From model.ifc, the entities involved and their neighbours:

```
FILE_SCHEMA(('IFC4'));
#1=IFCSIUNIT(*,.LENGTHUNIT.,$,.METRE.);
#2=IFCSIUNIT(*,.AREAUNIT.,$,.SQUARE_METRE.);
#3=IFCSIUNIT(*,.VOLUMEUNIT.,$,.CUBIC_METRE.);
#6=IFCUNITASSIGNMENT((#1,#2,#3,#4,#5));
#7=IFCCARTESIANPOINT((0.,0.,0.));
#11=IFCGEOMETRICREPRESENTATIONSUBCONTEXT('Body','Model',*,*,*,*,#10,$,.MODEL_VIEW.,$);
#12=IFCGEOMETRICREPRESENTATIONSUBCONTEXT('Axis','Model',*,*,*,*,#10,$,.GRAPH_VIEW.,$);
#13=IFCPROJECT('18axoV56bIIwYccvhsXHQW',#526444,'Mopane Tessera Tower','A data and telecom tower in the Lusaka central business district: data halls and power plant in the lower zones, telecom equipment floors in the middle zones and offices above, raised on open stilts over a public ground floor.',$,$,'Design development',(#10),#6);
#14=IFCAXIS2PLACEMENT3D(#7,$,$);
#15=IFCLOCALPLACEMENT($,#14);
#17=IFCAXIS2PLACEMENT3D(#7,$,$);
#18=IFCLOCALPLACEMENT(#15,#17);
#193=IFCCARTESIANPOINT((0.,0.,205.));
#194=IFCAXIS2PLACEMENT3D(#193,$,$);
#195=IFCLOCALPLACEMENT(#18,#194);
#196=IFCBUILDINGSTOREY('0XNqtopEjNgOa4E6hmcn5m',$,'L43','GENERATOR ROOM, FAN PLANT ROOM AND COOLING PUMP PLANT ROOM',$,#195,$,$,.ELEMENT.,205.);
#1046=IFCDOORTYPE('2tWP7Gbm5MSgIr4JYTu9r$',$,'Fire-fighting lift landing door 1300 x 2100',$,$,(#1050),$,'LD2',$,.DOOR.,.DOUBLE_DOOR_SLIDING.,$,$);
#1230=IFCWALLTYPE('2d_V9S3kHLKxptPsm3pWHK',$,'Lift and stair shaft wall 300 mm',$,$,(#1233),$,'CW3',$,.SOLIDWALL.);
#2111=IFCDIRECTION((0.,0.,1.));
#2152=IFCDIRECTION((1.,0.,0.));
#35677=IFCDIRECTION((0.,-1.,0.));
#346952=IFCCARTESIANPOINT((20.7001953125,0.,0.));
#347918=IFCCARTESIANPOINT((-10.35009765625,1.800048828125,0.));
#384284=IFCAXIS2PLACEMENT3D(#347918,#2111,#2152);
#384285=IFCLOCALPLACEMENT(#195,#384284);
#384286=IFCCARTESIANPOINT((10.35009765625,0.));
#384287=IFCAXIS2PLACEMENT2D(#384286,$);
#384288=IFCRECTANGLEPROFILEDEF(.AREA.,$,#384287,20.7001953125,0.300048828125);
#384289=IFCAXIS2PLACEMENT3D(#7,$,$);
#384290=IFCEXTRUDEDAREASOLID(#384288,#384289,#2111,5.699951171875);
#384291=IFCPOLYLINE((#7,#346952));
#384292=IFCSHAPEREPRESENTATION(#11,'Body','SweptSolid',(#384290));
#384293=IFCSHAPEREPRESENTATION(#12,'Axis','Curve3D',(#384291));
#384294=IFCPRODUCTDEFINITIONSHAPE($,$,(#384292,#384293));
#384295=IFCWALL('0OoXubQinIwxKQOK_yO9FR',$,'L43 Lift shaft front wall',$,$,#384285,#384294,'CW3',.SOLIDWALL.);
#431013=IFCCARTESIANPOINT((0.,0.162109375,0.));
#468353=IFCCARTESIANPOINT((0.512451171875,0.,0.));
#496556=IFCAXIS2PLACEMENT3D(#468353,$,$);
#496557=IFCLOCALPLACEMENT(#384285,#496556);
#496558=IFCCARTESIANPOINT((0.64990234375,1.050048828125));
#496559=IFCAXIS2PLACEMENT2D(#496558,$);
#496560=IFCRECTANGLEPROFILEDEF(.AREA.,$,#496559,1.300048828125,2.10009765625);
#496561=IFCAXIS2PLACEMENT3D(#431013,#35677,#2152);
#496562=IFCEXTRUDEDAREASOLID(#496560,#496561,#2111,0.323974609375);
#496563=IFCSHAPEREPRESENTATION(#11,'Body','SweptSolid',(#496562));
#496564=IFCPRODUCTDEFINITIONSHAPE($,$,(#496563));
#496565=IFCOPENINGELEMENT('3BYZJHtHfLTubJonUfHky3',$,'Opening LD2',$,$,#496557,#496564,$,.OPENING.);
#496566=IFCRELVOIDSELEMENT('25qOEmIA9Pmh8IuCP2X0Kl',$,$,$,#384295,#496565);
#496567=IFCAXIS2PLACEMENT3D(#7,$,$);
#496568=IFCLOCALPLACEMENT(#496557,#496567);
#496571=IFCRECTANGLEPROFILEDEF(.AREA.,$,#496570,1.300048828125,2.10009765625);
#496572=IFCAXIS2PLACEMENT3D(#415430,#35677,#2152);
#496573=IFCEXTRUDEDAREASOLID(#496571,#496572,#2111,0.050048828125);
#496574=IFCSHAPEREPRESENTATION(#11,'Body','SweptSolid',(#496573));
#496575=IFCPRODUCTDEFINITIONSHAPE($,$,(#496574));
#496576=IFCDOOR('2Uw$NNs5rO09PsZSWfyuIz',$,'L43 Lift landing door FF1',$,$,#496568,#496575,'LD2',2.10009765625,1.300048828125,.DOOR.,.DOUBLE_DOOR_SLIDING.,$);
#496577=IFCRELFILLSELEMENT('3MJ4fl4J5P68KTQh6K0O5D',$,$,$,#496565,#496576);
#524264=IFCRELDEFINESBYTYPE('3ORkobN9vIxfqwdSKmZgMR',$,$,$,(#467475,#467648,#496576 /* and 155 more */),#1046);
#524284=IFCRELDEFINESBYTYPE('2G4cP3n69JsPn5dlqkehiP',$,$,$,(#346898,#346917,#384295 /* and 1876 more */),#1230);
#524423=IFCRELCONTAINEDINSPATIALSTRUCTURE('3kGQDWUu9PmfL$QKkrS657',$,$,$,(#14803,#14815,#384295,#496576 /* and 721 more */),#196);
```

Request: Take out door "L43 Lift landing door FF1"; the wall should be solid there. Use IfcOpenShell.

```python
import ifcopenshell
import ifcopenshell.api.feature
import ifcopenshell.api.root
import ifcopenshell.geom
import ifcopenshell.util.shape

model = ifcopenshell.open("model.ifc")
settings = ifcopenshell.geom.settings()


def volume(element):
    """Net volume in cubic metres, openings subtracted."""
    shape = ifcopenshell.geom.create_shape(settings, element)
    return ifcopenshell.util.shape.get_volume(shape.geometry)


door = model.by_id(496576)
opening = door.FillsVoids[0].RelatingOpeningElement
wall = opening.VoidsElements[0].RelatingBuildingElement
before = volume(wall)

ifcopenshell.api.root.remove_product(model, product=door)
ifcopenshell.api.feature.remove_feature(model, feature=opening)

after = volume(wall)

print(f"wall volume {before:.3f} -> {after:.3f} m3")

model.write("model_updated.ifc")
```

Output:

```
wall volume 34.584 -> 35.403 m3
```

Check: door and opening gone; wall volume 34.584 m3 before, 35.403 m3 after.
